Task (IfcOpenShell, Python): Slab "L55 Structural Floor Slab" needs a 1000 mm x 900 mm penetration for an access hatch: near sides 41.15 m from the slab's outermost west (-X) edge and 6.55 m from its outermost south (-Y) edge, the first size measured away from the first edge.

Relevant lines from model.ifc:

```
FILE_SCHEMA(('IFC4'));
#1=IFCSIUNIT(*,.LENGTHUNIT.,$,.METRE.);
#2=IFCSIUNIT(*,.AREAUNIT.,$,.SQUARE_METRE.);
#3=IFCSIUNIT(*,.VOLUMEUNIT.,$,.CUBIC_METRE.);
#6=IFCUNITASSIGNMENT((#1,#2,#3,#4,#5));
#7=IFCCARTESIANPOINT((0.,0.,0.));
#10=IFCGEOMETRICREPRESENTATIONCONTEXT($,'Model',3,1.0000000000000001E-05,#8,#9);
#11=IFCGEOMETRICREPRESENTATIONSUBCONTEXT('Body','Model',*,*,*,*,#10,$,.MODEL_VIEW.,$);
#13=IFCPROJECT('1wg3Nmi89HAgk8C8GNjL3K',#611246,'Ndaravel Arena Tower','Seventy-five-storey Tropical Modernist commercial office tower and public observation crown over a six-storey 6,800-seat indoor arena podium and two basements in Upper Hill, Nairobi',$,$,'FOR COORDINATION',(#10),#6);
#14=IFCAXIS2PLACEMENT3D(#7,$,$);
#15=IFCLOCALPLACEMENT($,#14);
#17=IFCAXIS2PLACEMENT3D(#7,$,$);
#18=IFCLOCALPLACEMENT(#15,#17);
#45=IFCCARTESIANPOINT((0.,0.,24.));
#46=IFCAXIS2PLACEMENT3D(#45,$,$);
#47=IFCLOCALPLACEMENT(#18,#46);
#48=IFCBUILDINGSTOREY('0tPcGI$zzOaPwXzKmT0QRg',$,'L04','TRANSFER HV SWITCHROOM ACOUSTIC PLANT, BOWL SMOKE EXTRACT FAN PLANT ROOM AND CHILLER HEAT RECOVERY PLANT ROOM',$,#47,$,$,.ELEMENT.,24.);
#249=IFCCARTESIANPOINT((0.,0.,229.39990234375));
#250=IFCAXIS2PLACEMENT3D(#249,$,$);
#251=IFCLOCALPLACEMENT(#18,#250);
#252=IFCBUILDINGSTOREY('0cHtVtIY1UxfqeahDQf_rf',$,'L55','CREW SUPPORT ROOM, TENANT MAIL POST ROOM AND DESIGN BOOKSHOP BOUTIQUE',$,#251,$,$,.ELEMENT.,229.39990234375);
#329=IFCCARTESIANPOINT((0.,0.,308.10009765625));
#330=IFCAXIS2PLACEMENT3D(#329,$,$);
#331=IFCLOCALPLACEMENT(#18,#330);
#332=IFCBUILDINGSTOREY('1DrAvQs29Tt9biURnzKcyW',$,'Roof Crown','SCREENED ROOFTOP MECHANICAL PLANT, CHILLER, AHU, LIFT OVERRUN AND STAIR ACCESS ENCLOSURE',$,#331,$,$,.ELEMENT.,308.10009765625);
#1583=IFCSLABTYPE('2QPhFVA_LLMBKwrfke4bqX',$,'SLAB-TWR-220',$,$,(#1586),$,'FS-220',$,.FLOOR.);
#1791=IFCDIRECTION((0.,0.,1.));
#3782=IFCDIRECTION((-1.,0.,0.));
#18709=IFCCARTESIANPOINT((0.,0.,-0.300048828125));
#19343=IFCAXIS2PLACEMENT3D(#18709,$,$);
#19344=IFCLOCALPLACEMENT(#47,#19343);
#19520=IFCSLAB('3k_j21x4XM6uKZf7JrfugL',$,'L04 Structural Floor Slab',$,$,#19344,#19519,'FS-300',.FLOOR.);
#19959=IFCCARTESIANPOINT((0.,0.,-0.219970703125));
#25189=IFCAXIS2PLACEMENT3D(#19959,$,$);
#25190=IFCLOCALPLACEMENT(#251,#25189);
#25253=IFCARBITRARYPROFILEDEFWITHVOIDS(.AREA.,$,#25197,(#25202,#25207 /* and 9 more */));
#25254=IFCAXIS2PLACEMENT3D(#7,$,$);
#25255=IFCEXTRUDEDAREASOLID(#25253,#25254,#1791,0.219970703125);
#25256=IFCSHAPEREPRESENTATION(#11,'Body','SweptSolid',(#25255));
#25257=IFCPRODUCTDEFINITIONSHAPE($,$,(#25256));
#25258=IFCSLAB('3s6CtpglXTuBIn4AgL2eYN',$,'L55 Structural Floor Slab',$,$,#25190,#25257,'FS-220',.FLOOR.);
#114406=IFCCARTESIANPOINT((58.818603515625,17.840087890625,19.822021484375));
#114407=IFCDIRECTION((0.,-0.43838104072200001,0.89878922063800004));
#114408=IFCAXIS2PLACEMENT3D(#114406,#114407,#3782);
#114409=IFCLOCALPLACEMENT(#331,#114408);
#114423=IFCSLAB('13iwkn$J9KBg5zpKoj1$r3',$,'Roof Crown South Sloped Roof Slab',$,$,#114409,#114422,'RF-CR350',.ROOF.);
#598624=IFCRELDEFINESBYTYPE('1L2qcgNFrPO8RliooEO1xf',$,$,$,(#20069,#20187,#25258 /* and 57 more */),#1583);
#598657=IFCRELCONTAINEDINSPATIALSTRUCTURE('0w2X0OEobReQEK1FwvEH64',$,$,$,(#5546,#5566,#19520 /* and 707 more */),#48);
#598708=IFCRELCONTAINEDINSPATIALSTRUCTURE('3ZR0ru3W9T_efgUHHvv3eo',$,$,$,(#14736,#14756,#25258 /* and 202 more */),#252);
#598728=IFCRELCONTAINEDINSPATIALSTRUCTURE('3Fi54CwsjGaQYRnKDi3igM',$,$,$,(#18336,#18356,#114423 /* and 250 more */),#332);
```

```python
import numpy as np
import ifcopenshell
import ifcopenshell.api.feature
import ifcopenshell.api.geometry
import ifcopenshell.api.root
import ifcopenshell.geom
import ifcopenshell.util.placement
import ifcopenshell.util.representation
import ifcopenshell.util.shape
import ifcopenshell.util.unit

model = ifcopenshell.open("model.ifc")
unit_scale = ifcopenshell.util.unit.calculate_unit_scale(model)
settings = ifcopenshell.geom.settings()


def volume(element):
    """Net volume in cubic metres, openings subtracted."""
    shape = ifcopenshell.geom.create_shape(settings, element)
    return ifcopenshell.util.shape.get_volume(shape.geometry)


slab = model.by_guid("3s6CtpglXTuBIn4AgL2eYN")
before = volume(slab)

# Extent in the slab's own axes, in metres. The edges named are its -X and -Y sides.
slab_shape = ifcopenshell.geom.create_shape(settings, slab)
vertices = ifcopenshell.util.shape.get_vertices(slab_shape.geometry)
x_min, y_min, bottom = vertices.min(axis=0)
top = vertices[:, 2].max()

opening = ifcopenshell.api.root.create_entity(model, ifc_class="IfcOpeningElement", name="Access hatch opening", predefined_type="OPENING")
context = ifcopenshell.util.representation.get_context(model, "Model", "Body", "MODEL_VIEW")
width, depth = 1, 0.9
outline = [(0.0, 0.0), (width, 0.0), (width, depth), (0.0, depth), (0.0, 0.0)]
# Overshoot both faces by 50 mm so the cut is clean.
shape = ifcopenshell.api.geometry.add_slab_representation(
    model, context=context, depth=top - bottom + 0.1, polyline=outline
)
ifcopenshell.api.geometry.assign_representation(model, product=opening, representation=shape)

matrix = ifcopenshell.util.placement.get_local_placement(slab.ObjectPlacement)
matrix[:, 3] = matrix @ np.append(np.array([x_min + 41.15, y_min + 6.55, bottom - 0.05]) / unit_scale, 1.0)
ifcopenshell.api.geometry.edit_object_placement(model, product=opening, matrix=matrix, is_si=False)
ifcopenshell.api.feature.add_feature(model, feature=opening, element=slab)

after = volume(slab)

print(f"slab volume {before:.3f} -> {after:.3f} m3")

model.write("model_updated.ifc")
```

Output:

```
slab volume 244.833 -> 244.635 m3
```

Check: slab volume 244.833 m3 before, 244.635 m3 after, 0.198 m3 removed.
